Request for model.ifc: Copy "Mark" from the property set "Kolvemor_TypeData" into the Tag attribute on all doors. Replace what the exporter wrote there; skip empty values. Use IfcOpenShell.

First a look at what the model holds.

```python
import ifcopenshell
import ifcopenshell.util.element

model = ifcopenshell.open("model.ifc")
print(model.schema)
doors = model.by_type("IfcDoor")
print(len(doors), "doors")
for e in doors[:8]:
    source = ifcopenshell.util.element.get_pset(e, "Kolvemor_TypeData", "Mark")
    target = e.Tag
    print(e.id(), repr(source), repr(target), sep=" | ")
```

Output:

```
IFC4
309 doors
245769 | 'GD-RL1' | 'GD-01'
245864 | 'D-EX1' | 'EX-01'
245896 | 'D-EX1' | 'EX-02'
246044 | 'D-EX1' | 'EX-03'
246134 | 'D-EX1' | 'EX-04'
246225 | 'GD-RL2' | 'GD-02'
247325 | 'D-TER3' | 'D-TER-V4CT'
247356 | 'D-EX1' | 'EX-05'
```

```python
import ifcopenshell
import ifcopenshell.util.element

model = ifcopenshell.open("model.ifc")

count = 0
for e in model.by_type("IfcDoor"):
    value = ifcopenshell.util.element.get_pset(e, "Kolvemor_TypeData", "Mark")
    current = e.Tag
    if not value or not value.strip() or current == value:
        continue
    e.Tag = value
    count += 1

print(count, "doors updated")

model.write("model-out.ifc")
```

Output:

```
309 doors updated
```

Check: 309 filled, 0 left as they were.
